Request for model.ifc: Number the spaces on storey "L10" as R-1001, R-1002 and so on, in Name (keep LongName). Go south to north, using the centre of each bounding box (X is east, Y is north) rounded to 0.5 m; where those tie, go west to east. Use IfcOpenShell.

First a look at what the model holds.

```python
import ifcopenshell
import ifcopenshell.util.element
import ifcopenshell.util.placement

model = ifcopenshell.open("model.ifc")
print(model.schema)
storey = next(s for s in model.by_type("IfcBuildingStorey") if s.Name == "L10")
spaces = [e for e in ifcopenshell.util.element.get_decomposition(storey) if e.is_a("IfcSpace")]
for e in sorted(spaces, key=lambda e: e.id()):
    origin = ifcopenshell.util.placement.get_local_placement(e.ObjectPlacement)[:3, 3]
    print(e.id(), e.Name, e.LongName, origin.round(2) + 0.0, sep=" | ")
```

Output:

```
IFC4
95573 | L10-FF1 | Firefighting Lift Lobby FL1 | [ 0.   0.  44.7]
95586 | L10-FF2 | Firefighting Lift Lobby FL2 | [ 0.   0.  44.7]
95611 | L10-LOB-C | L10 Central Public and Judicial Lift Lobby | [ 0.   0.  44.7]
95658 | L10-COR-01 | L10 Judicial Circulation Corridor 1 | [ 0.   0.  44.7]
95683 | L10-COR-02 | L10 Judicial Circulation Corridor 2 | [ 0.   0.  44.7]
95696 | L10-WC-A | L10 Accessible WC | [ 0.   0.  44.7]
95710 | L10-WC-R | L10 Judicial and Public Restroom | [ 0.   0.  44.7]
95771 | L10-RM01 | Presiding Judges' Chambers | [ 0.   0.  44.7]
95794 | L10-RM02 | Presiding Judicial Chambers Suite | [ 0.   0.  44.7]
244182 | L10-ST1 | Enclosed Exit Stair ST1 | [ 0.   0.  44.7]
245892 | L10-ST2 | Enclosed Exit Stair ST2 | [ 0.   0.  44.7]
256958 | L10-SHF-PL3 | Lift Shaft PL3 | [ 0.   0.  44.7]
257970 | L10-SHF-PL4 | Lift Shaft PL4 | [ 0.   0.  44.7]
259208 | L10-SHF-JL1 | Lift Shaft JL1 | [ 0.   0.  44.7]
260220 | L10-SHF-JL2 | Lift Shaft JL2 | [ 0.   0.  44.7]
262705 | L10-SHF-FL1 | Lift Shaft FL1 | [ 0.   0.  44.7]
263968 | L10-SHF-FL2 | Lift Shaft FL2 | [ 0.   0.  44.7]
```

```python
import ifcopenshell
import ifcopenshell.geom
import ifcopenshell.util.element
import ifcopenshell.util.shape

model = ifcopenshell.open("model.ifc")
settings = ifcopenshell.geom.settings()
settings.set("use-world-coords", True)


def centre(element):
    shape = ifcopenshell.geom.create_shape(settings, element)
    return ifcopenshell.util.shape.get_bbox_centroid(shape.geometry)


storey = next(s for s in model.by_type("IfcBuildingStorey") if s.Name == "L10")
spaces = [e for e in ifcopenshell.util.element.get_decomposition(storey) if e.is_a("IfcSpace")]

# Insertion points can sit at a corner or the storey origin, so sort by the geometry (in metres).
centres = {e: centre(e) for e in spaces}
spaces.sort(key=lambda e: (round(centres[e][1] / 0.5), centres[e][0]))

for i, e in enumerate(spaces, start=1):
    number = f"R-10{i:02d}"
    e.Name = number
    print(e.id(), number)

model.write("model_rev.ifc")
```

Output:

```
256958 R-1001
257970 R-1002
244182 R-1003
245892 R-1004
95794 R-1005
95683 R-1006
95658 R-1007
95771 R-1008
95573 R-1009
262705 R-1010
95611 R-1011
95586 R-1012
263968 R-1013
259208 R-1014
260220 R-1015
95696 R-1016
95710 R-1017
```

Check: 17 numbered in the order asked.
